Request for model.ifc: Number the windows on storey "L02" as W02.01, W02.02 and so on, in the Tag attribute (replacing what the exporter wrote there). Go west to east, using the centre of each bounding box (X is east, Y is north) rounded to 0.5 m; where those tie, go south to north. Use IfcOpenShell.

First a look at what the model holds.

```python
import ifcopenshell
import ifcopenshell.util.element
import ifcopenshell.util.placement

model = ifcopenshell.open("model.ifc")
print(model.schema)
storey = next(s for s in model.by_type("IfcBuildingStorey") if s.Name == "L02")
windows = [e for e in ifcopenshell.util.element.get_decomposition(storey) if e.is_a("IfcWindow")]
for e in sorted(windows, key=lambda e: e.id()):
    origin = ifcopenshell.util.placement.get_local_placement(e.ObjectPlacement)[:3, 3]
    print(e.id(), e.Tag, e.Name, origin.round(2) + 0.0, sep=" | ")
```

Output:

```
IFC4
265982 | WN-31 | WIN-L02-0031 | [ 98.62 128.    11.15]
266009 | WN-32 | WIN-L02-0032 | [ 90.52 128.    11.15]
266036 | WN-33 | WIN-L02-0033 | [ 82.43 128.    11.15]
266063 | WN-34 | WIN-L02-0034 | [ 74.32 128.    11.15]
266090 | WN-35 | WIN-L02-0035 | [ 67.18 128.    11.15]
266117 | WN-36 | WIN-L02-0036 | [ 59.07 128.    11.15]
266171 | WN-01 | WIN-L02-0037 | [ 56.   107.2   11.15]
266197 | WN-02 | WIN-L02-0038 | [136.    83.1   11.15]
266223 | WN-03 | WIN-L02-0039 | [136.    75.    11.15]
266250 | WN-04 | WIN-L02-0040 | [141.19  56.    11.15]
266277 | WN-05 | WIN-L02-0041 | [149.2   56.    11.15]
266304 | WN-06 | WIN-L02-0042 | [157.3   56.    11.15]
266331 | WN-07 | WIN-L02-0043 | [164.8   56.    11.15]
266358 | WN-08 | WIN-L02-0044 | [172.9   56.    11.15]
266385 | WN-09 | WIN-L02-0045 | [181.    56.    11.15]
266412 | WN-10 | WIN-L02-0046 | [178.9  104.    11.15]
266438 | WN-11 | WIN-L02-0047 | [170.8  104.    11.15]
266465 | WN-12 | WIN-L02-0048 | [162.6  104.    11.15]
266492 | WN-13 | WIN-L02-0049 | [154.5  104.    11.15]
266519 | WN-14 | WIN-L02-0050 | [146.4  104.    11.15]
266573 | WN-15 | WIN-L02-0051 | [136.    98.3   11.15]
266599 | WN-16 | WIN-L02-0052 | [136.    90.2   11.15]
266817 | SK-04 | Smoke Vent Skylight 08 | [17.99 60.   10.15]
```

```python
import ifcopenshell
import ifcopenshell.geom
import ifcopenshell.util.element
import ifcopenshell.util.shape

model = ifcopenshell.open("model.ifc")
settings = ifcopenshell.geom.settings()
settings.set("use-world-coords", True)


def centre(element):
    shape = ifcopenshell.geom.create_shape(settings, element)
    return ifcopenshell.util.shape.get_bbox_centroid(shape.geometry)


storey = next(s for s in model.by_type("IfcBuildingStorey") if s.Name == "L02")
windows = [e for e in ifcopenshell.util.element.get_decomposition(storey) if e.is_a("IfcWindow")]

# Insertion points can sit at a corner or the storey origin, so sort by the geometry (in metres).
centres = {e: centre(e) for e in windows}
windows.sort(key=lambda e: (round(centres[e][0] / 0.5), centres[e][1]))

for i, e in enumerate(windows, start=1):
    number = f"W02.{i:02d}"
    e.Tag = number
    print(e.id(), number)

model.write("model-out.ifc")
```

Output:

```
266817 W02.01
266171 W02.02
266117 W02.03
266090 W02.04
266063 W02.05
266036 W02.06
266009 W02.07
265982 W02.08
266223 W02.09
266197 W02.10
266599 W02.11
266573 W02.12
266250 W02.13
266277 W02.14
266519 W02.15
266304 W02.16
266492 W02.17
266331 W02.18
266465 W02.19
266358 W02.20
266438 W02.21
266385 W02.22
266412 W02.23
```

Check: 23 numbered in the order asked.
